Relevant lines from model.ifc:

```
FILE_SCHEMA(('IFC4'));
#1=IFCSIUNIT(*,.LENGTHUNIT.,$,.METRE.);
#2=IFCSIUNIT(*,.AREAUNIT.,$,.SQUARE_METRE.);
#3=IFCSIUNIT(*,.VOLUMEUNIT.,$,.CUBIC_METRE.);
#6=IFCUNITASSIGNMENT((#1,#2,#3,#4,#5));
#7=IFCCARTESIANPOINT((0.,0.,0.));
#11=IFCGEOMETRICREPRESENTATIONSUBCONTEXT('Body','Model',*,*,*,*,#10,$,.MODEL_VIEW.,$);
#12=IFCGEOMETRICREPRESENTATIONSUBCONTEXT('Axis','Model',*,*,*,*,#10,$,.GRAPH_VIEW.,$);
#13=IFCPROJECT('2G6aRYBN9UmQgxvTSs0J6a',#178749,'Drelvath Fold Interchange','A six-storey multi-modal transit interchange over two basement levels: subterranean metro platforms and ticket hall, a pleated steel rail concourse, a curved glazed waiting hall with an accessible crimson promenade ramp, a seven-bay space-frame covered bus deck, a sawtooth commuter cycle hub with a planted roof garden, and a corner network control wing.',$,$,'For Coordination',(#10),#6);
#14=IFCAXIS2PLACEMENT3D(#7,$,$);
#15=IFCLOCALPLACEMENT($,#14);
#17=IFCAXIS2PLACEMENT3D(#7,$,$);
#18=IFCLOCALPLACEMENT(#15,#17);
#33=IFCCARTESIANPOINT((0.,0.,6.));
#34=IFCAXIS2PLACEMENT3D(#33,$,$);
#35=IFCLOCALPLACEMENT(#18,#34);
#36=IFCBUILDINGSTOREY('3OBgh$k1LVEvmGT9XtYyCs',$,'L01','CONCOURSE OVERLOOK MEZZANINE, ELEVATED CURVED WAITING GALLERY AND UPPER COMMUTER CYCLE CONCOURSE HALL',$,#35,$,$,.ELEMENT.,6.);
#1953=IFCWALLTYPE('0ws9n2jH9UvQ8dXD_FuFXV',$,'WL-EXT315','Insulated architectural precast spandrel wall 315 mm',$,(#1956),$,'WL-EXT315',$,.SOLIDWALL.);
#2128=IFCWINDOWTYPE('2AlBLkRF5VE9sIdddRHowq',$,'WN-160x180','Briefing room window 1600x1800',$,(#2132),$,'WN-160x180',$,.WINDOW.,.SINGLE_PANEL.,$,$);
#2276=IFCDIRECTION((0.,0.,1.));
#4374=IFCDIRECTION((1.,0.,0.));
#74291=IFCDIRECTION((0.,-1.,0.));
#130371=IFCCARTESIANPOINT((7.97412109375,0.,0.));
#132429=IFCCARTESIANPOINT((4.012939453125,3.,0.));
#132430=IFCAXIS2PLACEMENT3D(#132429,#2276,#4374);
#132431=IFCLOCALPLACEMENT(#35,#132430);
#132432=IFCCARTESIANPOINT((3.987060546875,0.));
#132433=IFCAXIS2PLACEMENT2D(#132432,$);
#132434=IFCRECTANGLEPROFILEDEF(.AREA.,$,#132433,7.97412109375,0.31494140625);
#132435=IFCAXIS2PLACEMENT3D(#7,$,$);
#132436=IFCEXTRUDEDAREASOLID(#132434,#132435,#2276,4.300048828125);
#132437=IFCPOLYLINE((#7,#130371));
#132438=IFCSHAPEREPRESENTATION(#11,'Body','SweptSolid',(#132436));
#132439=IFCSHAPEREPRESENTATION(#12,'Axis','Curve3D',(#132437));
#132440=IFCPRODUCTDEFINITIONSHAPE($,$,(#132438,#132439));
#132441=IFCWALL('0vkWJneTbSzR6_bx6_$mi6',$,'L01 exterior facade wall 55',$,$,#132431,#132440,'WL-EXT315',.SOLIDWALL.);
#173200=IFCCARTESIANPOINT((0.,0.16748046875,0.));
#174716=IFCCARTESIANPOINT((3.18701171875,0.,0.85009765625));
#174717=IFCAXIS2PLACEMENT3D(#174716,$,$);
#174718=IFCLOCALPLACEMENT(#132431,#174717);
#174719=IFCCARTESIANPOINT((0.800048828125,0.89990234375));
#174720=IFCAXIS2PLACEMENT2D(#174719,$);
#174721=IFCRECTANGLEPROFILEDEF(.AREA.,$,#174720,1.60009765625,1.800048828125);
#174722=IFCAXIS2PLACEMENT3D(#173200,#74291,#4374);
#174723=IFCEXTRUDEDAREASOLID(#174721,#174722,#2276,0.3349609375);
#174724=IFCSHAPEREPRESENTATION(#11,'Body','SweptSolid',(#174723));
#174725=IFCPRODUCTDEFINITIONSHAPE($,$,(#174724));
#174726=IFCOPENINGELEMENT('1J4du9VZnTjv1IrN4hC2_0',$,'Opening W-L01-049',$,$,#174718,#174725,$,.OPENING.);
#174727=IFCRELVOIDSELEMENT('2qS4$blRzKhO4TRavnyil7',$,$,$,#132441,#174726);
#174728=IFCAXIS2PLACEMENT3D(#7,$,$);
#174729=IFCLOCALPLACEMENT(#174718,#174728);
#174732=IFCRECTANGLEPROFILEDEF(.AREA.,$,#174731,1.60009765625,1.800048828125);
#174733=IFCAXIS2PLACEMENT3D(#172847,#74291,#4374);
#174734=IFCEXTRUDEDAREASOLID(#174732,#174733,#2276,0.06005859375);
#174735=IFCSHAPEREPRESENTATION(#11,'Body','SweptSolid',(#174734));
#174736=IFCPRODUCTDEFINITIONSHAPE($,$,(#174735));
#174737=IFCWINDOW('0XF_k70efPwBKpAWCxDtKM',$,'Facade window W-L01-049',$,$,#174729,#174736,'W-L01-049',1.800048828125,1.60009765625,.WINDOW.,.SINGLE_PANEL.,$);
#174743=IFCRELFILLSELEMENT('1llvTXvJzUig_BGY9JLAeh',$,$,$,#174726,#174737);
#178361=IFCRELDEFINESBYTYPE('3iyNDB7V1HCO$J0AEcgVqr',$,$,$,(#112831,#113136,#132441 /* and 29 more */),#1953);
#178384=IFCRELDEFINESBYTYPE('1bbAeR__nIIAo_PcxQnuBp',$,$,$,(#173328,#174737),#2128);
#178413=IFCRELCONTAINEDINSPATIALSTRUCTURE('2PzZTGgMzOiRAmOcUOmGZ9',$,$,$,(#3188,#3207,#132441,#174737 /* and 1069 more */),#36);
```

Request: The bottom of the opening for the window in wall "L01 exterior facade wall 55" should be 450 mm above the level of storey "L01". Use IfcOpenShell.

```python
import numpy as np
import ifcopenshell
import ifcopenshell.api.geometry
import ifcopenshell.geom
import ifcopenshell.util.element
import ifcopenshell.util.placement
import ifcopenshell.util.shape
import ifcopenshell.util.unit

model = ifcopenshell.open("model.ifc")
unit_scale = ifcopenshell.util.unit.calculate_unit_scale(model)

window = model.by_id(174737)
opening = window.FillsVoids[0].RelatingOpeningElement
storey = ifcopenshell.util.element.get_container(window, ifc_class="IfcBuildingStorey")
level = ifcopenshell.util.placement.get_local_placement(storey.ObjectPlacement)[2, 3]

# The opening's origin need not be at the sill, so measure its lowest point.
shape = ifcopenshell.geom.create_shape(ifcopenshell.geom.settings(), opening)
bottom = ifcopenshell.util.shape.get_shape_bottom_elevation(shape, shape.geometry) / unit_scale
dz = level + 0.45 / unit_scale - bottom

shift = np.array([0.0, 0.0, dz])
# The window is placed relative to its opening, so it follows when the opening moves.
matrix = ifcopenshell.util.placement.get_local_placement(opening.ObjectPlacement)
matrix[:3, 3] += shift
ifcopenshell.api.geometry.edit_object_placement(
    model, product=opening, matrix=matrix, is_si=False, should_transform_children=True
)

print(f"moved by {dz * unit_scale:+.3f} m")

model.write("model_rev.ifc")
```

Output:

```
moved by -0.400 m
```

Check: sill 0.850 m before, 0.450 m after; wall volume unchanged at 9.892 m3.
